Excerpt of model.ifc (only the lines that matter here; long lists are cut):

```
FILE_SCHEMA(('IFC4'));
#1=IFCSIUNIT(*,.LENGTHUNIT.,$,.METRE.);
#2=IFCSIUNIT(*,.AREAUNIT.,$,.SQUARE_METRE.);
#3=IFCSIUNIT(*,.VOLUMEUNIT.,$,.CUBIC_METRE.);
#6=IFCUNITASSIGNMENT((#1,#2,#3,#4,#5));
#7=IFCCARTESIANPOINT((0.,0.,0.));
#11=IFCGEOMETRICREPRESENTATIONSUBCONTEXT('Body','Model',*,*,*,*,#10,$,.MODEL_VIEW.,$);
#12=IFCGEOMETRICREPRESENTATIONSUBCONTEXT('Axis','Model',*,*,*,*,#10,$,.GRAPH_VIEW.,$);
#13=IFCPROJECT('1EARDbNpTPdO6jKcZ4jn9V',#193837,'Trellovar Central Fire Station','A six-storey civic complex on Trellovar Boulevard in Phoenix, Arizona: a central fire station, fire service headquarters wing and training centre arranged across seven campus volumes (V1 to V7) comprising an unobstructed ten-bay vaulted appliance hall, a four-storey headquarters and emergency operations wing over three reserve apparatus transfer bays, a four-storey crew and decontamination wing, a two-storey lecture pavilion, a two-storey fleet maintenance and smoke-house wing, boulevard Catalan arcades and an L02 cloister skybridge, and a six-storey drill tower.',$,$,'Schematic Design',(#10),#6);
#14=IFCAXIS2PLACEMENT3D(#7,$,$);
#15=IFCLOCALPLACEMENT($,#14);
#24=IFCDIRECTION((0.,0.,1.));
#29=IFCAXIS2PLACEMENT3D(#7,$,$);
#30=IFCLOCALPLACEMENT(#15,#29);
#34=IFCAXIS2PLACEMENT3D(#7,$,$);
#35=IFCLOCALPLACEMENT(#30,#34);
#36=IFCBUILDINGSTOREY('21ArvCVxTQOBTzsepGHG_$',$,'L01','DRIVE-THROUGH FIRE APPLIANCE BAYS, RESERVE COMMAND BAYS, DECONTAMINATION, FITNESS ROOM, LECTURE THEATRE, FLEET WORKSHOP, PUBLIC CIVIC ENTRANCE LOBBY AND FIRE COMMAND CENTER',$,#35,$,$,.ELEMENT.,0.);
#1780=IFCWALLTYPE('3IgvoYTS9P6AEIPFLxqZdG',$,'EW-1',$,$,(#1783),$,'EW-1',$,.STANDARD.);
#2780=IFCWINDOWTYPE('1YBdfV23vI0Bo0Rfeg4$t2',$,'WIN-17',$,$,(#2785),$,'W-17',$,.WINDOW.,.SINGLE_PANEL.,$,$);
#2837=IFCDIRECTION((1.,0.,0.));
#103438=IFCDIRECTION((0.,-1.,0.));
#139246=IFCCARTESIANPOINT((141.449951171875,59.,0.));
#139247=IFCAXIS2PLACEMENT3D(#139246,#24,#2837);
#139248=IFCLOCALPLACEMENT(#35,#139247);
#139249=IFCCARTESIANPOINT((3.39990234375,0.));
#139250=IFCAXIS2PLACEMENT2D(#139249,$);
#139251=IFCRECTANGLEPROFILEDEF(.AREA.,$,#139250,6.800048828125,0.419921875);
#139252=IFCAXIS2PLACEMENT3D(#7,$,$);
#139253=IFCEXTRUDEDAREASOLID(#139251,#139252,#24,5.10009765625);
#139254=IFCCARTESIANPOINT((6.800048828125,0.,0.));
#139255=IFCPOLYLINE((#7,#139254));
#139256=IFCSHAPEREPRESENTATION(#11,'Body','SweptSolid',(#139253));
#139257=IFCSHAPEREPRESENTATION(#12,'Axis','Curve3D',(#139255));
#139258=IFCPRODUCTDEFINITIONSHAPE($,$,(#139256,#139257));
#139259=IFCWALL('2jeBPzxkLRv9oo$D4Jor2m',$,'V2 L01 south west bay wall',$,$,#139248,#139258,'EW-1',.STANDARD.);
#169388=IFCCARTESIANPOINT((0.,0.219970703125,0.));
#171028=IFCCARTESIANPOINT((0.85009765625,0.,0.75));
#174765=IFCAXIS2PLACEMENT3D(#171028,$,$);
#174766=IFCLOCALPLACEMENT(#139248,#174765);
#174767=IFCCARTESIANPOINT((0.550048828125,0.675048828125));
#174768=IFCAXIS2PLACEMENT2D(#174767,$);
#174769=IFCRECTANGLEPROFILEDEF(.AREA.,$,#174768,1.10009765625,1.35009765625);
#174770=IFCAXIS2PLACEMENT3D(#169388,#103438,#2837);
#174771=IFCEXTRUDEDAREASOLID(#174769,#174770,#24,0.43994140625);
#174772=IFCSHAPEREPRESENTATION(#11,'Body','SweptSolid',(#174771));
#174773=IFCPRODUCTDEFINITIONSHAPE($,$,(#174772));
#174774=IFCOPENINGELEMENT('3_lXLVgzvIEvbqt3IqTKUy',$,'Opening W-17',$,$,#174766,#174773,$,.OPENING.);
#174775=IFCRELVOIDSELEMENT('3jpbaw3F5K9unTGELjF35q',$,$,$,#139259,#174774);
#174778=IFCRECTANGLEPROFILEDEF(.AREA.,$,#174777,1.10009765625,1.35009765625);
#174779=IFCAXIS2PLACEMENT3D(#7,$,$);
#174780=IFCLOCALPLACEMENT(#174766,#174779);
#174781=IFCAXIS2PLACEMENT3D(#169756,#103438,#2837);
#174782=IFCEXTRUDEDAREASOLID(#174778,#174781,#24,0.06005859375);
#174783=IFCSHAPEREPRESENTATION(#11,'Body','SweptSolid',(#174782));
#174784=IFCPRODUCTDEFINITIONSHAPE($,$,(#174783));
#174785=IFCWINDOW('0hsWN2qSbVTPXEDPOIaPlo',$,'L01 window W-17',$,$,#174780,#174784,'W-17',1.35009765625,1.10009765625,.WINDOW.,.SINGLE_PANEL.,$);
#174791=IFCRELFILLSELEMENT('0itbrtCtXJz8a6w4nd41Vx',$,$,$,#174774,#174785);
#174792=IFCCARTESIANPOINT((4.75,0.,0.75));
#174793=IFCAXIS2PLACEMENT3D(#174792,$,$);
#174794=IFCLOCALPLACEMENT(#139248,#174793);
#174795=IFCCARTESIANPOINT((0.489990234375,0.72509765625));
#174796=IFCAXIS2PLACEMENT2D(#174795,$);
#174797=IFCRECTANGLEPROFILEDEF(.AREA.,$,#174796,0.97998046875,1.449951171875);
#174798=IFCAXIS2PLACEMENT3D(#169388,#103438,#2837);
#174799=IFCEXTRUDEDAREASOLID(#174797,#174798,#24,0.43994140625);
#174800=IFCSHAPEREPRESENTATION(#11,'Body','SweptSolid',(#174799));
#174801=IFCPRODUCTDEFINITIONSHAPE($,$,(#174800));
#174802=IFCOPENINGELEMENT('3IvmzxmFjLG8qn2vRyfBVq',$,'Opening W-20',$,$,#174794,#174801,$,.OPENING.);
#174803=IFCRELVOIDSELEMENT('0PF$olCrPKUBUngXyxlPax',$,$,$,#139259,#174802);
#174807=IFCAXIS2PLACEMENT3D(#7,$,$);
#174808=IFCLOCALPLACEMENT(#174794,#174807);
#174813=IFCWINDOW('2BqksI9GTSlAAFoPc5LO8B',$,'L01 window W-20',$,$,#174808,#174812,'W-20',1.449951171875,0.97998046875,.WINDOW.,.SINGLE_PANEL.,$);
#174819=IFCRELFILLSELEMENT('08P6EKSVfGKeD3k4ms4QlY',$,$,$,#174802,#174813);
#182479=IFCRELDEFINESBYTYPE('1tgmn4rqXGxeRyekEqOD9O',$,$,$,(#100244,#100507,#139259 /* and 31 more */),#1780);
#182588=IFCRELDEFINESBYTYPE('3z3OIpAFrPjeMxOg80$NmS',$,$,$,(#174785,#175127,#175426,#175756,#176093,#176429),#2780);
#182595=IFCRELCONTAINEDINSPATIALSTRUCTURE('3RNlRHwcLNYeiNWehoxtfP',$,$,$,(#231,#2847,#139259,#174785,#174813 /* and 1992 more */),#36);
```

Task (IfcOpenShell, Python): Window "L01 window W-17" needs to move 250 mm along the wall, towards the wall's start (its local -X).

```python
import ifcopenshell
import ifcopenshell.api.geometry
import ifcopenshell.util.placement
import ifcopenshell.util.unit

model = ifcopenshell.open("model.ifc")
unit_scale = ifcopenshell.util.unit.calculate_unit_scale(model)

window = model.by_guid("0hsWN2qSbVTPXEDPOIaPlo")
opening = window.FillsVoids[0].RelatingOpeningElement
wall = opening.VoidsElements[0].RelatingBuildingElement

wall_matrix = ifcopenshell.util.placement.get_local_placement(wall.ObjectPlacement)
shift = wall_matrix[:3, 0] * -0.25 / unit_scale
before = ifcopenshell.util.placement.get_local_placement(window.ObjectPlacement)[:3, 3].copy()

# The window is placed relative to its opening, so it follows when the opening moves.
matrix = ifcopenshell.util.placement.get_local_placement(opening.ObjectPlacement)
matrix[:3, 3] += shift
ifcopenshell.api.geometry.edit_object_placement(
    model, product=opening, matrix=matrix, is_si=False, should_transform_children=True
)

after = ifcopenshell.util.placement.get_local_placement(window.ObjectPlacement)[:3, 3]
print("window moved by", (after - before).round(3) + 0.0)

model.write("model_v2.ifc")
```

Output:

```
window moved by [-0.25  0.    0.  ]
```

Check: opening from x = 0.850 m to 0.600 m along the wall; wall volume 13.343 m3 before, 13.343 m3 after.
